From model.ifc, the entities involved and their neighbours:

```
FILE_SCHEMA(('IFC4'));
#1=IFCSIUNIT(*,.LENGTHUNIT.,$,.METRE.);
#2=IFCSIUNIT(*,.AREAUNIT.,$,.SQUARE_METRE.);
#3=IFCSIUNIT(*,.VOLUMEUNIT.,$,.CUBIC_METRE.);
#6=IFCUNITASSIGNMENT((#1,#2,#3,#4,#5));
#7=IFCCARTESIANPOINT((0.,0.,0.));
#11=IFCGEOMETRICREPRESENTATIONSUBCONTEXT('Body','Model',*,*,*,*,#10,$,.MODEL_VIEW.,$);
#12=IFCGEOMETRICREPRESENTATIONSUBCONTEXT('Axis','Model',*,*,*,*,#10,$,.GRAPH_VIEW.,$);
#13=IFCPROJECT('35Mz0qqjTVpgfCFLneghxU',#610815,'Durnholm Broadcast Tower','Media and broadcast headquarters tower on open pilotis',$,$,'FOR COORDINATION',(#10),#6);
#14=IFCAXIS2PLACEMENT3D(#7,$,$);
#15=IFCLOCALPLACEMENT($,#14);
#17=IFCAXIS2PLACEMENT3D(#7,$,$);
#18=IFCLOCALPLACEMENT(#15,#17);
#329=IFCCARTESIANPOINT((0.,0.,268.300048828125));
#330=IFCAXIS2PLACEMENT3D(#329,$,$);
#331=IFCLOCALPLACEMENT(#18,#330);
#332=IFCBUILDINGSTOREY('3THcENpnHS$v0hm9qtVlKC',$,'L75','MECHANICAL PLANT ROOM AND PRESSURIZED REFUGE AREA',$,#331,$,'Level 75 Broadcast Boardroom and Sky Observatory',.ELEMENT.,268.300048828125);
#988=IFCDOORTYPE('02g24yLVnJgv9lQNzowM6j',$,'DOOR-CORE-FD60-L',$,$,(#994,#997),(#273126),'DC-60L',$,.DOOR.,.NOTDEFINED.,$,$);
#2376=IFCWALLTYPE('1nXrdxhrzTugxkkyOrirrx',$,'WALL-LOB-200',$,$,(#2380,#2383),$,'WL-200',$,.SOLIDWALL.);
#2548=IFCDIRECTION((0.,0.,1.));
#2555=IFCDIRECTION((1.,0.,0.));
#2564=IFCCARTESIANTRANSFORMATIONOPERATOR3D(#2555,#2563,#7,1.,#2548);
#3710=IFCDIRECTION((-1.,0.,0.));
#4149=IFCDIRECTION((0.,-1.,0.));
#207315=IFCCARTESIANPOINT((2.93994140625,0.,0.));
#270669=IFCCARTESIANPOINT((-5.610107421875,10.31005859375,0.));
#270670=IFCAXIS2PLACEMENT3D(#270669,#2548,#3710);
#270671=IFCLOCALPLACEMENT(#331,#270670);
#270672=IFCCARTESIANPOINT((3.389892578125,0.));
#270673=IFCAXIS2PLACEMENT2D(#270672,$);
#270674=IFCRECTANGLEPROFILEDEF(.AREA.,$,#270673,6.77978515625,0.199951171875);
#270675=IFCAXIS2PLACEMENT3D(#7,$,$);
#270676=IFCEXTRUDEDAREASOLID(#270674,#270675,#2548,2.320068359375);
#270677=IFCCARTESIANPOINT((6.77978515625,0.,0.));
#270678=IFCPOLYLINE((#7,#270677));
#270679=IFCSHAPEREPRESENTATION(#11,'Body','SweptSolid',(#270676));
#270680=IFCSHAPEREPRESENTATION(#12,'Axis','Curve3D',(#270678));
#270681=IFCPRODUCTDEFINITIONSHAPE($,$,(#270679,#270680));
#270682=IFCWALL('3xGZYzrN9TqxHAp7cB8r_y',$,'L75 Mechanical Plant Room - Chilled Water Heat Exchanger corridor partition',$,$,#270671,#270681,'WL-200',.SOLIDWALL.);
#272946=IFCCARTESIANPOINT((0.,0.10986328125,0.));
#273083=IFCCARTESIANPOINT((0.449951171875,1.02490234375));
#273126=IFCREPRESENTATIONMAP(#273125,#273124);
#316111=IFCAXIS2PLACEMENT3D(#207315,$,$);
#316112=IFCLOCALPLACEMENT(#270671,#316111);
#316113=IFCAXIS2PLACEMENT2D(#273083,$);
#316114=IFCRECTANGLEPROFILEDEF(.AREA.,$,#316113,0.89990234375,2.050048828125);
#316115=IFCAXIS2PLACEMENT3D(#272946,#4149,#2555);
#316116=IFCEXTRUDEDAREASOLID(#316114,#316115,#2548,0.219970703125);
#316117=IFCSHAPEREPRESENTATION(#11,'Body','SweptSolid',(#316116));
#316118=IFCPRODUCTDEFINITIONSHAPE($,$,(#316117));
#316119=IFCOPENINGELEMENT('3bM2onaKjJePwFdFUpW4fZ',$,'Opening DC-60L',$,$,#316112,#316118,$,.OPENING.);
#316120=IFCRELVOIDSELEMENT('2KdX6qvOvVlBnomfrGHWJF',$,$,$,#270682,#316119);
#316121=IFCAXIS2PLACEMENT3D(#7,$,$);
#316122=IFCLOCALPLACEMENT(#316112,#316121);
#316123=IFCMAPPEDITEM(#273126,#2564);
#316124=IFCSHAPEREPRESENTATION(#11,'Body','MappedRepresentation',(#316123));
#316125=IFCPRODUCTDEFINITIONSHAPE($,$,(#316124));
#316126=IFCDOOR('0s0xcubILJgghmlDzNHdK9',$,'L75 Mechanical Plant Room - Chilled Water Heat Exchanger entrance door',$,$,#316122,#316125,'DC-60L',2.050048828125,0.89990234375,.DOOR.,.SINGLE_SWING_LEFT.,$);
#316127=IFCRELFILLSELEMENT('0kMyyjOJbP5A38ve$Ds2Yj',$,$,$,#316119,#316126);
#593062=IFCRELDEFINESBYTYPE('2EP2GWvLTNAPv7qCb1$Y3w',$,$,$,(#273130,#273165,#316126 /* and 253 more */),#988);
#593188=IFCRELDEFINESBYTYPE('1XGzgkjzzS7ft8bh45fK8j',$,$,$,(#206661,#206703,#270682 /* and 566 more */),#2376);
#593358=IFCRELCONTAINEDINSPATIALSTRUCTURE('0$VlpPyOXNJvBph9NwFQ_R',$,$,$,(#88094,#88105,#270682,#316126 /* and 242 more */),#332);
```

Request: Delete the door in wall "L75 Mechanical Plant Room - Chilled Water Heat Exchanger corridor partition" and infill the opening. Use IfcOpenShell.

```python
import ifcopenshell
import ifcopenshell.api.feature
import ifcopenshell.api.root
import ifcopenshell.geom
import ifcopenshell.util.shape

model = ifcopenshell.open("model.ifc")
settings = ifcopenshell.geom.settings()


def volume(element):
    """Net volume in cubic metres, openings subtracted."""
    shape = ifcopenshell.geom.create_shape(settings, element)
    return ifcopenshell.util.shape.get_volume(shape.geometry)


door = model.by_id(316126)
opening = door.FillsVoids[0].RelatingOpeningElement
wall = opening.VoidsElements[0].RelatingBuildingElement
before = volume(wall)

ifcopenshell.api.root.remove_product(model, product=door)
ifcopenshell.api.feature.remove_feature(model, feature=opening)

after = volume(wall)

print(f"wall volume {before:.3f} -> {after:.3f} m3")

model.write("model_rev.ifc")
```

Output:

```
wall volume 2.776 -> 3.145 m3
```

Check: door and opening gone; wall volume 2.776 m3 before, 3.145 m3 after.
